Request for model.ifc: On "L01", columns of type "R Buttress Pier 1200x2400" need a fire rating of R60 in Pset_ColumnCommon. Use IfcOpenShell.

First a look at what the model holds.

```python
import ifcopenshell
import ifcopenshell.util.element

model = ifcopenshell.open("model.ifc")
print(model.schema)
storey = next(s for s in model.by_type("IfcBuildingStorey") if s.Name == "L01")
columns = [e for e in ifcopenshell.util.element.get_decomposition(storey) if e.is_a("IfcColumn")]
seen = {}
for e in columns:
    element_type = ifcopenshell.util.element.get_type(e)
    key = (element_type.Name if element_type != e and element_type else None, ifcopenshell.util.element.get_pset(e, "Pset_ColumnCommon", "FireRating"))
    seen[key] = seen.get(key, 0) + 1
for (name, value), count in sorted(seen.items(), key=str):
    print(count, "x", name, "|", value)
```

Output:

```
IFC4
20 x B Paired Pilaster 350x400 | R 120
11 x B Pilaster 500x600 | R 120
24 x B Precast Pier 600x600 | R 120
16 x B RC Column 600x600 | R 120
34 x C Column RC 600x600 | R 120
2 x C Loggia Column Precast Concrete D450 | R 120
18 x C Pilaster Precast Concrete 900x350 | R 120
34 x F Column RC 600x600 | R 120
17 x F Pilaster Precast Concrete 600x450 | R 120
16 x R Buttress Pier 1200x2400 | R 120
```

```python
import ifcopenshell
import ifcopenshell.api.pset
import ifcopenshell.util.element

model = ifcopenshell.open("model.ifc")

storey = next(s for s in model.by_type("IfcBuildingStorey") if s.Name == "L01")
columns = [e for e in ifcopenshell.util.element.get_decomposition(storey) if e.is_a("IfcColumn")]

count = 0
for e in columns:
    element_type = ifcopenshell.util.element.get_type(e)
    if element_type in (None, e) or element_type.Name != "R Buttress Pier 1200x2400":
        continue
    # add_pset returns the element's existing set when there is one.
    pset = ifcopenshell.api.pset.add_pset(model, product=e, name="Pset_ColumnCommon")
    ifcopenshell.api.pset.edit_pset(model, pset=pset, properties={"FireRating": "R60"})
    count += 1

print(count, "columns updated")

model.write("model_rev.ifc")
```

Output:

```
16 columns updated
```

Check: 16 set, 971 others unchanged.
